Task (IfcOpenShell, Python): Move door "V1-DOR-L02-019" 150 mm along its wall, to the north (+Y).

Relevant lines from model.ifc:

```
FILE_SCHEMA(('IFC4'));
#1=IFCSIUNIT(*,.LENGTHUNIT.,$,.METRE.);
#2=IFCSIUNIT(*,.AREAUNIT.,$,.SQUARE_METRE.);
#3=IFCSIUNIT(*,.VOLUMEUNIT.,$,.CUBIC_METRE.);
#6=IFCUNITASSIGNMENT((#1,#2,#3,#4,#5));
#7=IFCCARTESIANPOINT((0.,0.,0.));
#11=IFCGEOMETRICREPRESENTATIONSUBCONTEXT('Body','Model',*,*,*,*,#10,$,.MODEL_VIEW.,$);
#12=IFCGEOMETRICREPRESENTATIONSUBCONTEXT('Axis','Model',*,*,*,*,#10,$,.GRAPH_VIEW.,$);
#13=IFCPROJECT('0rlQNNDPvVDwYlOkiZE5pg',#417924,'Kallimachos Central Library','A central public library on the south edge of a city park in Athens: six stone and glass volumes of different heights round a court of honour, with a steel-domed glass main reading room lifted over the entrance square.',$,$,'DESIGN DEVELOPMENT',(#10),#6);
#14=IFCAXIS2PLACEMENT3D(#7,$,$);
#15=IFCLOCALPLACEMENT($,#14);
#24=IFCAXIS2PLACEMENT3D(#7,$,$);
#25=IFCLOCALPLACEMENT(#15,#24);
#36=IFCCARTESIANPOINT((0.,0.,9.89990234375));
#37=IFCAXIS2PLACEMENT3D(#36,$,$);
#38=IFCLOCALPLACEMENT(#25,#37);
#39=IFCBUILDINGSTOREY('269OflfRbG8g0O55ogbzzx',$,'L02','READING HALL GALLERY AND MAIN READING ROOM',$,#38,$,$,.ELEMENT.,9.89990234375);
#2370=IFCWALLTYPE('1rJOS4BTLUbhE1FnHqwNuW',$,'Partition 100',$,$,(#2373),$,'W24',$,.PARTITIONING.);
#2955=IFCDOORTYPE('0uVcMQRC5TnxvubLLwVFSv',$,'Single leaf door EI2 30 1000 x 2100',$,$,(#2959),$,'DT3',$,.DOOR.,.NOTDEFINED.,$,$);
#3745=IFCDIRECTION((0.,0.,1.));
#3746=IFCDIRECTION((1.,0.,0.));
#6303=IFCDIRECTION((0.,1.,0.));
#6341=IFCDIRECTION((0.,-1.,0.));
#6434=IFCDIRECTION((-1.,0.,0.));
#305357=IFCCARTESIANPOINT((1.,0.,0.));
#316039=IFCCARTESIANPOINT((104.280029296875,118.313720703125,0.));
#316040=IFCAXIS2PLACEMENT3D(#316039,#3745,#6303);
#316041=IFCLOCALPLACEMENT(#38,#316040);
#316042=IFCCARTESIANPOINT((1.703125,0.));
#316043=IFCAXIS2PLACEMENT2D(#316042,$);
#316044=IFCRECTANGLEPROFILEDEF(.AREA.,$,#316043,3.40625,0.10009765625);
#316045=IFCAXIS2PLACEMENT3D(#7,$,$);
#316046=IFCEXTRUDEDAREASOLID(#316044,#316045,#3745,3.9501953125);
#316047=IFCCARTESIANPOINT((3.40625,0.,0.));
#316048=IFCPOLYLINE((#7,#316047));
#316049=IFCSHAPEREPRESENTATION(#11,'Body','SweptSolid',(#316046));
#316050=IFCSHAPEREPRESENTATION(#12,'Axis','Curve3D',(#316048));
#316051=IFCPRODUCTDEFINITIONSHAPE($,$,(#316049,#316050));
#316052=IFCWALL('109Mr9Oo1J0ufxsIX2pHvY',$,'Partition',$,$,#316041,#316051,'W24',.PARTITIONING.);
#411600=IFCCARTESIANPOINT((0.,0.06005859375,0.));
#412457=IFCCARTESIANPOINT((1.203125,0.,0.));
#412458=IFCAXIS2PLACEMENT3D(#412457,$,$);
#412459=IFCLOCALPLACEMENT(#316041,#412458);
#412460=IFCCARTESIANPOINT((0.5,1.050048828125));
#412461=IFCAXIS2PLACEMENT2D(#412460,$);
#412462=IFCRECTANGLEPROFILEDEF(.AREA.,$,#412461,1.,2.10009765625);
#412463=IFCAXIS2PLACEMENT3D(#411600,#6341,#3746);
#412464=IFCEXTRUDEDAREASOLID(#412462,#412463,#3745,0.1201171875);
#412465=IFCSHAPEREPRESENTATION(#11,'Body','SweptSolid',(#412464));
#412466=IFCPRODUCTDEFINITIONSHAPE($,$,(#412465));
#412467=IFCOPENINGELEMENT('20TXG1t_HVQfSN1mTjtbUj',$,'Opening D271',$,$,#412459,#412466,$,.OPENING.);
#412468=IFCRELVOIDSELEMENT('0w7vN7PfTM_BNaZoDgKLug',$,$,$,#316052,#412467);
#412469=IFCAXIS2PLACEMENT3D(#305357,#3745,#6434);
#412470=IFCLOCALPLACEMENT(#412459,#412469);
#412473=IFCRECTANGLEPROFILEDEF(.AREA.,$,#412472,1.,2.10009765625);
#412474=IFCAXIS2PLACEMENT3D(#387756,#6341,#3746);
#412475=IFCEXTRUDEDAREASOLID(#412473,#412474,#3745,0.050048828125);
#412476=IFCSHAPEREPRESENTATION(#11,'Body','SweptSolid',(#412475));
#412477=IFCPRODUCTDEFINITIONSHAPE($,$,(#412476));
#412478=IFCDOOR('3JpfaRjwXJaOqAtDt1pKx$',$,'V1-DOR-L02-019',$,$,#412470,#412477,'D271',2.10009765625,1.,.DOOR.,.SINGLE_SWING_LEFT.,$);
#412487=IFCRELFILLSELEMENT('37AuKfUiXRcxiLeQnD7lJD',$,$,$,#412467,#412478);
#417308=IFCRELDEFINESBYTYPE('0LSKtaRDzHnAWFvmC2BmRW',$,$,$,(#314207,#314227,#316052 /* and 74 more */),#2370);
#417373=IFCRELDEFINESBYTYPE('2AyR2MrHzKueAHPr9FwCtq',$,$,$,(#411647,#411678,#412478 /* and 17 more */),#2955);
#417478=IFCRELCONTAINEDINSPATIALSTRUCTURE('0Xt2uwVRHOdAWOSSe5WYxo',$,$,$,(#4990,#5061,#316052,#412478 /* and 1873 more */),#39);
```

```python
import ifcopenshell
import ifcopenshell.api.geometry
import ifcopenshell.util.placement

model = ifcopenshell.open("model.ifc")

door = model.by_guid("3JpfaRjwXJaOqAtDt1pKx$")
opening = door.FillsVoids[0].RelatingOpeningElement
wall = opening.VoidsElements[0].RelatingBuildingElement

wall_matrix = ifcopenshell.util.placement.get_local_placement(wall.ObjectPlacement)
shift = wall_matrix[:3, 0] * 0.15
before = ifcopenshell.util.placement.get_local_placement(door.ObjectPlacement)[:3, 3].copy()

# The door is placed relative to its opening, so it follows when the opening moves.
matrix = ifcopenshell.util.placement.get_local_placement(opening.ObjectPlacement)
matrix[:3, 3] += shift
ifcopenshell.api.geometry.edit_object_placement(
    model, product=opening, matrix=matrix, is_si=False, should_transform_children=True
)

after = ifcopenshell.util.placement.get_local_placement(door.ObjectPlacement)[:3, 3]
print("door moved by", (after - before).round(3) + 0.0)

model.write("model_edited.ifc")
```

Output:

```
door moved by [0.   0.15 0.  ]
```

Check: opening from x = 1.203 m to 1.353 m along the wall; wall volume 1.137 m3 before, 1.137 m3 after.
